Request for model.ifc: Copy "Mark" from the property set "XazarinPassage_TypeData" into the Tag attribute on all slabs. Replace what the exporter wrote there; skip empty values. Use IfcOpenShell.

First a look at what the model holds.

```python
import ifcopenshell
import ifcopenshell.util.element

model = ifcopenshell.open("model.ifc")
print(model.schema)
slabs = model.by_type("IfcSlab")
print(len(slabs), "slabs")
for e in slabs[:8]:
    source = ifcopenshell.util.element.get_pset(e, "XazarinPassage_TypeData", "Mark")
    target = e.Tag
    print(e.id(), repr(source), repr(target), sep=" | ")
```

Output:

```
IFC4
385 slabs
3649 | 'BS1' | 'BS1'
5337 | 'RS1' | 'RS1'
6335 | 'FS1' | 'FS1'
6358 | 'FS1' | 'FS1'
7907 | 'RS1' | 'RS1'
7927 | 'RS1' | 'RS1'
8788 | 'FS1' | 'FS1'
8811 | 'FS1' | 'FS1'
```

```python
import ifcopenshell
import ifcopenshell.util.element

model = ifcopenshell.open("model.ifc")

count = 0
for e in model.by_type("IfcSlab"):
    value = ifcopenshell.util.element.get_pset(e, "XazarinPassage_TypeData", "Mark")
    current = e.Tag
    if not value or not value.strip() or current == value:
        continue
    e.Tag = value
    count += 1

print(count, "slabs updated")

model.write("model_v2.ifc")
```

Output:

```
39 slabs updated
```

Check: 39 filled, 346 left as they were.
